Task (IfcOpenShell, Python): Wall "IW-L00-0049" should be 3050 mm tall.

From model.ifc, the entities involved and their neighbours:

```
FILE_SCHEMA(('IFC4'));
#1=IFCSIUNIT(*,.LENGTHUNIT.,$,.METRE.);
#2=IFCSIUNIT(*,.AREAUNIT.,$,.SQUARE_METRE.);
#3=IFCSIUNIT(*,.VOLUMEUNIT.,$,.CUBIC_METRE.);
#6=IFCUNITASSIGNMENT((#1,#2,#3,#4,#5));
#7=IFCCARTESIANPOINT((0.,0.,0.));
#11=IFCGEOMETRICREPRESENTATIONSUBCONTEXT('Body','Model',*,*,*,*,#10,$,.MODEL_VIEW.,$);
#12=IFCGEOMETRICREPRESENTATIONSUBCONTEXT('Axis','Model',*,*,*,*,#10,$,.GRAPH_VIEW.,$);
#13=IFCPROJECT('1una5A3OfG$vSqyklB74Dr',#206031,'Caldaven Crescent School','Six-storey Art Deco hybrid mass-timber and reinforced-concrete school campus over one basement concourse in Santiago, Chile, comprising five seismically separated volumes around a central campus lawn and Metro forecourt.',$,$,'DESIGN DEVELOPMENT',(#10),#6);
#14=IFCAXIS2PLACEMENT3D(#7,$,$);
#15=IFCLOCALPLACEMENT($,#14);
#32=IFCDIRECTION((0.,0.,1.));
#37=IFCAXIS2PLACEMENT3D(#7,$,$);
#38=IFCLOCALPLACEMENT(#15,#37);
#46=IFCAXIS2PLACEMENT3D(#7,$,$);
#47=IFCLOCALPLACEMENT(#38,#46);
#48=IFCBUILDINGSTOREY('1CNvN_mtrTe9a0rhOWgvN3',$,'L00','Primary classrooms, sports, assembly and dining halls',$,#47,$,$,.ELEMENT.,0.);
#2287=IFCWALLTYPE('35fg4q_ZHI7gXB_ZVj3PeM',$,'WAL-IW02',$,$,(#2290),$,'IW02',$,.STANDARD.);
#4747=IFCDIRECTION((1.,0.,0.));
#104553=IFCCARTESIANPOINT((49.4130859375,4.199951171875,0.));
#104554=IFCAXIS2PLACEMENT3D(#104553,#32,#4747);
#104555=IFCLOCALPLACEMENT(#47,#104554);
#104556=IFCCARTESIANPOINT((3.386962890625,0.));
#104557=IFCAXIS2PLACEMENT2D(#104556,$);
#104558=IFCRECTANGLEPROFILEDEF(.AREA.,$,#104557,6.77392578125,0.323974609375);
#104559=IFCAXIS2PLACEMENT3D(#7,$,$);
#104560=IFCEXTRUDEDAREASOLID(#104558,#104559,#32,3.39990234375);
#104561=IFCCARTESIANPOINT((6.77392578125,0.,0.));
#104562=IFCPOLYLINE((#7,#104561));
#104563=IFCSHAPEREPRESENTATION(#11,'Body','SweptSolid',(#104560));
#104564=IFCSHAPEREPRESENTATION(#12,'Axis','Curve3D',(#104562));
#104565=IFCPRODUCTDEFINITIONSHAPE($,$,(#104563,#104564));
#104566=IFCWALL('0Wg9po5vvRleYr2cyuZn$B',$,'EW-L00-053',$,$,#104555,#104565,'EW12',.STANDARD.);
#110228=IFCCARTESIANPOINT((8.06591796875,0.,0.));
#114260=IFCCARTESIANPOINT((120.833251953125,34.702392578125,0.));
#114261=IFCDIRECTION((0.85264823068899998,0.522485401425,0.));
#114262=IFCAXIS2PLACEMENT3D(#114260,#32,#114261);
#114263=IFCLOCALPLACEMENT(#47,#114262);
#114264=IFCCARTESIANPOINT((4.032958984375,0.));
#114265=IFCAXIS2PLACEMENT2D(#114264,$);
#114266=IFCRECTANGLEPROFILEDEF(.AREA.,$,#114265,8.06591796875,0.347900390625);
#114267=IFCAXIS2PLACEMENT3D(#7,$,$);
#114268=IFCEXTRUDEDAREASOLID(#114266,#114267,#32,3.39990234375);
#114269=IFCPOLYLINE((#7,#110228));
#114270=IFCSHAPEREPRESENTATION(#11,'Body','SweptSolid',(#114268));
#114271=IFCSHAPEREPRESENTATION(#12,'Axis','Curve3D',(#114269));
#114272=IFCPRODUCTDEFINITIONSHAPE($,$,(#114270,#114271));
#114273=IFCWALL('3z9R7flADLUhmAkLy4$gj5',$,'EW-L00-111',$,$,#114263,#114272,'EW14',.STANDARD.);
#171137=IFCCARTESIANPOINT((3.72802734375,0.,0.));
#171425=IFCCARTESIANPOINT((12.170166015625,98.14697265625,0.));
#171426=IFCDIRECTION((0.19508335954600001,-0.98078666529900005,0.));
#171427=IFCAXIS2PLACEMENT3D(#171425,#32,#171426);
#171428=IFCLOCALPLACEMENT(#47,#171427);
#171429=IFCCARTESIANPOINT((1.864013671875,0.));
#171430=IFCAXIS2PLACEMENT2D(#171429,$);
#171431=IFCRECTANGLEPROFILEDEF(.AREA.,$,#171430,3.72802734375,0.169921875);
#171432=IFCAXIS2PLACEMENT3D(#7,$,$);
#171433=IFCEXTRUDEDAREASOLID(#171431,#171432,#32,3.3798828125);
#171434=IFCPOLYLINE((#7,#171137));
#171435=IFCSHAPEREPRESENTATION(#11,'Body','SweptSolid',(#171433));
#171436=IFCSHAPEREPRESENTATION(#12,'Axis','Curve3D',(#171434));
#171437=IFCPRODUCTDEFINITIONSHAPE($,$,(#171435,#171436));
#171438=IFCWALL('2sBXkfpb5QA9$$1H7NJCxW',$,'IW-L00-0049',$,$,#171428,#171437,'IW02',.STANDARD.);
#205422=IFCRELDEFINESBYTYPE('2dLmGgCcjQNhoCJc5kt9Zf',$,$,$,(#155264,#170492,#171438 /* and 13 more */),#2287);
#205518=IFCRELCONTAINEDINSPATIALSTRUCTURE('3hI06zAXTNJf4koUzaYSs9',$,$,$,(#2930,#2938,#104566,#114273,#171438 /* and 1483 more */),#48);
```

```python
import ifcopenshell
import ifcopenshell.geom
import ifcopenshell.util.representation
import ifcopenshell.util.shape

model = ifcopenshell.open("model.ifc")
settings = ifcopenshell.geom.settings()


def volume(element):
    """Net volume in cubic metres, openings subtracted."""
    shape = ifcopenshell.geom.create_shape(settings, element)
    return ifcopenshell.util.shape.get_volume(shape.geometry)


wall = model.by_guid("2sBXkfpb5QA9$$1H7NJCxW")
before = volume(wall)

body = ifcopenshell.util.representation.get_representation(wall, "Model", "Body")
solid = body.Items[0]
old_height = solid.Depth
solid.Depth = 3.05
after = volume(wall)

print(f"height {old_height:g} -> {solid.Depth:g}, volume {before:.3f} -> {after:.3f} m3")

model.write("model_updated.ifc")
```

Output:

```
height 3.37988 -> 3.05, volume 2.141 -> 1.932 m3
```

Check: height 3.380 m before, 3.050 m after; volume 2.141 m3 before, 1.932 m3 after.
